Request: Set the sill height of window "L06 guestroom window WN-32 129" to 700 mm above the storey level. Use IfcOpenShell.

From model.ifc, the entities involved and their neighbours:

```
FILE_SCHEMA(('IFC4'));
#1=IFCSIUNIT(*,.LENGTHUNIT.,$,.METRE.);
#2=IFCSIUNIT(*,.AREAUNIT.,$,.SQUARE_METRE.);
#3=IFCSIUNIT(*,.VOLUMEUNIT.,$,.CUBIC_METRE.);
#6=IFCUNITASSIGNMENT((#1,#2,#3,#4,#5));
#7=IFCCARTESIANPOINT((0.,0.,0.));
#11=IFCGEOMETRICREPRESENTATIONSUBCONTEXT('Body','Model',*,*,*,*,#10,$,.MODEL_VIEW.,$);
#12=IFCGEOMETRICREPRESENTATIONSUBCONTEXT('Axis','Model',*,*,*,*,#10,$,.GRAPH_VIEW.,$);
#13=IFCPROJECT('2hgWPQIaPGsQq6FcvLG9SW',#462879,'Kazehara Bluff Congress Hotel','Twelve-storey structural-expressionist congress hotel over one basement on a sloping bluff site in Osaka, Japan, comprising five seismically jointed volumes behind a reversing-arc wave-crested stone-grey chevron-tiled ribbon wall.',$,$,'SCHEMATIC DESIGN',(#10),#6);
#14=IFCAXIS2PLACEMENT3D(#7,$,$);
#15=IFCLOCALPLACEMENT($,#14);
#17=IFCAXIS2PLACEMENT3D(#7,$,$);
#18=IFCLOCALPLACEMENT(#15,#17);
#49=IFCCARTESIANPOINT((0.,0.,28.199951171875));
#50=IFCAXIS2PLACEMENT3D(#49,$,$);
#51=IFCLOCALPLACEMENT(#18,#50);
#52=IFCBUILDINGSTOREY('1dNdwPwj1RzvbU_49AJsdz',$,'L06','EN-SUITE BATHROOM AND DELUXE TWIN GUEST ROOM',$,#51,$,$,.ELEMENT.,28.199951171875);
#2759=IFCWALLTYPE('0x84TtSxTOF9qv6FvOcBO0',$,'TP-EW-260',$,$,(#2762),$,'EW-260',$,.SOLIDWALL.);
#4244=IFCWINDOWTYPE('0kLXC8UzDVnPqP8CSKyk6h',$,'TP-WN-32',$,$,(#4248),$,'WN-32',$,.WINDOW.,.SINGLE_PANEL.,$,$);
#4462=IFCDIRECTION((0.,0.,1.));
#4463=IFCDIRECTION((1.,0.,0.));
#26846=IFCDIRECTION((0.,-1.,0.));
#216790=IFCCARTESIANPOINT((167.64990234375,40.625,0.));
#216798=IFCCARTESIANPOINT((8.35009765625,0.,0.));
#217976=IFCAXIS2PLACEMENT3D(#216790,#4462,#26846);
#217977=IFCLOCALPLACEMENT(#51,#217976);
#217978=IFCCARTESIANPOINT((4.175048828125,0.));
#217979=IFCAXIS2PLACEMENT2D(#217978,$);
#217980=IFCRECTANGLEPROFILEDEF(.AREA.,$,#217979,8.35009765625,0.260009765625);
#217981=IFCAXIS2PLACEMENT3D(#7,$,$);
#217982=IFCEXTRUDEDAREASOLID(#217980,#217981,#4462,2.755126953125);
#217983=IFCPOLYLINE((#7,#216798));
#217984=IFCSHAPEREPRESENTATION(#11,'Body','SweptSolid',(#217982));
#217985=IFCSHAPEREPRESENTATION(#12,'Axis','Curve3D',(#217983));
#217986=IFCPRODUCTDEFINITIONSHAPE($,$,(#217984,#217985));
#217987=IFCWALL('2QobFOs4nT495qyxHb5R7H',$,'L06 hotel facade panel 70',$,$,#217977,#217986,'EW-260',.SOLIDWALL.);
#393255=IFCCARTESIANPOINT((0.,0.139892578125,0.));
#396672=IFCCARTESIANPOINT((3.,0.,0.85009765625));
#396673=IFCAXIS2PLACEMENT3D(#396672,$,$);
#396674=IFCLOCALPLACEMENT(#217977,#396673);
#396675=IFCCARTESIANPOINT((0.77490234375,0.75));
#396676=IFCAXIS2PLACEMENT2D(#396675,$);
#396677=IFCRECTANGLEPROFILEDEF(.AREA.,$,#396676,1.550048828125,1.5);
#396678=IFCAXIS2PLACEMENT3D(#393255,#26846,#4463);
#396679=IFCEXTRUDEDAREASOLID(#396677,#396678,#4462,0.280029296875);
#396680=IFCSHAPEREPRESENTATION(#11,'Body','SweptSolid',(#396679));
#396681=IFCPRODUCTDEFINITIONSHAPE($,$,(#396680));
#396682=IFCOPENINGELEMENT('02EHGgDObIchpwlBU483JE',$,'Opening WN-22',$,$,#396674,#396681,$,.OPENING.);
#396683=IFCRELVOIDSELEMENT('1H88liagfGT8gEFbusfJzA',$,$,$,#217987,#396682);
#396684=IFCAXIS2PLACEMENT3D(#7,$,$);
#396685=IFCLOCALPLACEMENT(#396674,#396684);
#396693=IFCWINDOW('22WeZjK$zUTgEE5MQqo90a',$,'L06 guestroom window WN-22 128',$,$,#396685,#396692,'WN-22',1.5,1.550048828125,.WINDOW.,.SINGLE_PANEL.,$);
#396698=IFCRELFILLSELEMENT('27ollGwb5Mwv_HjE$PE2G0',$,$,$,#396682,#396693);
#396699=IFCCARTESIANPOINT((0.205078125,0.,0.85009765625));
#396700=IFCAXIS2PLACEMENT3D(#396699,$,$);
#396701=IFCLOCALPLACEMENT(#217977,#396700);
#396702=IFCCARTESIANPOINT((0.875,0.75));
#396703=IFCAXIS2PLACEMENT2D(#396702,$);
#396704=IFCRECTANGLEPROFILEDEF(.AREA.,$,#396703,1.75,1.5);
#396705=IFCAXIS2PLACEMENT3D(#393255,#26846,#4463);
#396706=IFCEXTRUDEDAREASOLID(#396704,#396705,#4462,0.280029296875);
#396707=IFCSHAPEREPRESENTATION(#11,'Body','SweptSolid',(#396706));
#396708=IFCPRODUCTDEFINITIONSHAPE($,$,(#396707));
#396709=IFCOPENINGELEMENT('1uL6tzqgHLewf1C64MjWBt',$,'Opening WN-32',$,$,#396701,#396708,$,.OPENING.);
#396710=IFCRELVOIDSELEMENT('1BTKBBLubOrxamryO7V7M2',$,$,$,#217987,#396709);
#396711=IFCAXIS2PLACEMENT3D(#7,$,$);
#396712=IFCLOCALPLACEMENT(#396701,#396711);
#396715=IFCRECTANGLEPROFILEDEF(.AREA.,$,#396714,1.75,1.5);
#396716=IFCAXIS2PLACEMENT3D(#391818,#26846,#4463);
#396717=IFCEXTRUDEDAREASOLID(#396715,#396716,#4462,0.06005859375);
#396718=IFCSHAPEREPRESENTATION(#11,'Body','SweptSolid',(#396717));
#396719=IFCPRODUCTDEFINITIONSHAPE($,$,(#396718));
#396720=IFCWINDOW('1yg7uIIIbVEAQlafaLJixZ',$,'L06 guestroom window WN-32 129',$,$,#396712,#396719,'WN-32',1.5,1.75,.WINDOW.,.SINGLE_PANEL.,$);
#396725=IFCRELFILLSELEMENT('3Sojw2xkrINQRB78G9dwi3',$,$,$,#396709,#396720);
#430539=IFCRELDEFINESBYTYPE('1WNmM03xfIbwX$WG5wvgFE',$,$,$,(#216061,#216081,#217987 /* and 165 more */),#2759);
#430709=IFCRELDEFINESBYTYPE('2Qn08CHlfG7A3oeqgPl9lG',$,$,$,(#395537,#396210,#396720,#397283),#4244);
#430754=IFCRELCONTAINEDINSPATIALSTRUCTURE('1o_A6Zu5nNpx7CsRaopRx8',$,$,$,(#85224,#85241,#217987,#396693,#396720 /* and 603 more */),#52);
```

```python
import numpy as np
import ifcopenshell
import ifcopenshell.api.geometry
import ifcopenshell.geom
import ifcopenshell.util.element
import ifcopenshell.util.placement
import ifcopenshell.util.shape
import ifcopenshell.util.unit

model = ifcopenshell.open("model.ifc")
unit_scale = ifcopenshell.util.unit.calculate_unit_scale(model)

window = model.by_id(396720)
opening = window.FillsVoids[0].RelatingOpeningElement
storey = ifcopenshell.util.element.get_container(window, ifc_class="IfcBuildingStorey")
level = ifcopenshell.util.placement.get_local_placement(storey.ObjectPlacement)[2, 3]

# The opening's origin need not be at the sill, so measure its lowest point.
shape = ifcopenshell.geom.create_shape(ifcopenshell.geom.settings(), opening)
bottom = ifcopenshell.util.shape.get_shape_bottom_elevation(shape, shape.geometry) / unit_scale
dz = level + 0.7 / unit_scale - bottom

shift = np.array([0.0, 0.0, dz])
# The window is placed relative to its opening, so it follows when the opening moves.
matrix = ifcopenshell.util.placement.get_local_placement(opening.ObjectPlacement)
matrix[:3, 3] += shift
ifcopenshell.api.geometry.edit_object_placement(
    model, product=opening, matrix=matrix, is_si=False, should_transform_children=True
)

print(f"moved by {dz * unit_scale:+.3f} m")

model.write("model_rev.ifc")
```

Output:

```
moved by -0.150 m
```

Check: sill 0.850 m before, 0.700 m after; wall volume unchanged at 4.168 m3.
